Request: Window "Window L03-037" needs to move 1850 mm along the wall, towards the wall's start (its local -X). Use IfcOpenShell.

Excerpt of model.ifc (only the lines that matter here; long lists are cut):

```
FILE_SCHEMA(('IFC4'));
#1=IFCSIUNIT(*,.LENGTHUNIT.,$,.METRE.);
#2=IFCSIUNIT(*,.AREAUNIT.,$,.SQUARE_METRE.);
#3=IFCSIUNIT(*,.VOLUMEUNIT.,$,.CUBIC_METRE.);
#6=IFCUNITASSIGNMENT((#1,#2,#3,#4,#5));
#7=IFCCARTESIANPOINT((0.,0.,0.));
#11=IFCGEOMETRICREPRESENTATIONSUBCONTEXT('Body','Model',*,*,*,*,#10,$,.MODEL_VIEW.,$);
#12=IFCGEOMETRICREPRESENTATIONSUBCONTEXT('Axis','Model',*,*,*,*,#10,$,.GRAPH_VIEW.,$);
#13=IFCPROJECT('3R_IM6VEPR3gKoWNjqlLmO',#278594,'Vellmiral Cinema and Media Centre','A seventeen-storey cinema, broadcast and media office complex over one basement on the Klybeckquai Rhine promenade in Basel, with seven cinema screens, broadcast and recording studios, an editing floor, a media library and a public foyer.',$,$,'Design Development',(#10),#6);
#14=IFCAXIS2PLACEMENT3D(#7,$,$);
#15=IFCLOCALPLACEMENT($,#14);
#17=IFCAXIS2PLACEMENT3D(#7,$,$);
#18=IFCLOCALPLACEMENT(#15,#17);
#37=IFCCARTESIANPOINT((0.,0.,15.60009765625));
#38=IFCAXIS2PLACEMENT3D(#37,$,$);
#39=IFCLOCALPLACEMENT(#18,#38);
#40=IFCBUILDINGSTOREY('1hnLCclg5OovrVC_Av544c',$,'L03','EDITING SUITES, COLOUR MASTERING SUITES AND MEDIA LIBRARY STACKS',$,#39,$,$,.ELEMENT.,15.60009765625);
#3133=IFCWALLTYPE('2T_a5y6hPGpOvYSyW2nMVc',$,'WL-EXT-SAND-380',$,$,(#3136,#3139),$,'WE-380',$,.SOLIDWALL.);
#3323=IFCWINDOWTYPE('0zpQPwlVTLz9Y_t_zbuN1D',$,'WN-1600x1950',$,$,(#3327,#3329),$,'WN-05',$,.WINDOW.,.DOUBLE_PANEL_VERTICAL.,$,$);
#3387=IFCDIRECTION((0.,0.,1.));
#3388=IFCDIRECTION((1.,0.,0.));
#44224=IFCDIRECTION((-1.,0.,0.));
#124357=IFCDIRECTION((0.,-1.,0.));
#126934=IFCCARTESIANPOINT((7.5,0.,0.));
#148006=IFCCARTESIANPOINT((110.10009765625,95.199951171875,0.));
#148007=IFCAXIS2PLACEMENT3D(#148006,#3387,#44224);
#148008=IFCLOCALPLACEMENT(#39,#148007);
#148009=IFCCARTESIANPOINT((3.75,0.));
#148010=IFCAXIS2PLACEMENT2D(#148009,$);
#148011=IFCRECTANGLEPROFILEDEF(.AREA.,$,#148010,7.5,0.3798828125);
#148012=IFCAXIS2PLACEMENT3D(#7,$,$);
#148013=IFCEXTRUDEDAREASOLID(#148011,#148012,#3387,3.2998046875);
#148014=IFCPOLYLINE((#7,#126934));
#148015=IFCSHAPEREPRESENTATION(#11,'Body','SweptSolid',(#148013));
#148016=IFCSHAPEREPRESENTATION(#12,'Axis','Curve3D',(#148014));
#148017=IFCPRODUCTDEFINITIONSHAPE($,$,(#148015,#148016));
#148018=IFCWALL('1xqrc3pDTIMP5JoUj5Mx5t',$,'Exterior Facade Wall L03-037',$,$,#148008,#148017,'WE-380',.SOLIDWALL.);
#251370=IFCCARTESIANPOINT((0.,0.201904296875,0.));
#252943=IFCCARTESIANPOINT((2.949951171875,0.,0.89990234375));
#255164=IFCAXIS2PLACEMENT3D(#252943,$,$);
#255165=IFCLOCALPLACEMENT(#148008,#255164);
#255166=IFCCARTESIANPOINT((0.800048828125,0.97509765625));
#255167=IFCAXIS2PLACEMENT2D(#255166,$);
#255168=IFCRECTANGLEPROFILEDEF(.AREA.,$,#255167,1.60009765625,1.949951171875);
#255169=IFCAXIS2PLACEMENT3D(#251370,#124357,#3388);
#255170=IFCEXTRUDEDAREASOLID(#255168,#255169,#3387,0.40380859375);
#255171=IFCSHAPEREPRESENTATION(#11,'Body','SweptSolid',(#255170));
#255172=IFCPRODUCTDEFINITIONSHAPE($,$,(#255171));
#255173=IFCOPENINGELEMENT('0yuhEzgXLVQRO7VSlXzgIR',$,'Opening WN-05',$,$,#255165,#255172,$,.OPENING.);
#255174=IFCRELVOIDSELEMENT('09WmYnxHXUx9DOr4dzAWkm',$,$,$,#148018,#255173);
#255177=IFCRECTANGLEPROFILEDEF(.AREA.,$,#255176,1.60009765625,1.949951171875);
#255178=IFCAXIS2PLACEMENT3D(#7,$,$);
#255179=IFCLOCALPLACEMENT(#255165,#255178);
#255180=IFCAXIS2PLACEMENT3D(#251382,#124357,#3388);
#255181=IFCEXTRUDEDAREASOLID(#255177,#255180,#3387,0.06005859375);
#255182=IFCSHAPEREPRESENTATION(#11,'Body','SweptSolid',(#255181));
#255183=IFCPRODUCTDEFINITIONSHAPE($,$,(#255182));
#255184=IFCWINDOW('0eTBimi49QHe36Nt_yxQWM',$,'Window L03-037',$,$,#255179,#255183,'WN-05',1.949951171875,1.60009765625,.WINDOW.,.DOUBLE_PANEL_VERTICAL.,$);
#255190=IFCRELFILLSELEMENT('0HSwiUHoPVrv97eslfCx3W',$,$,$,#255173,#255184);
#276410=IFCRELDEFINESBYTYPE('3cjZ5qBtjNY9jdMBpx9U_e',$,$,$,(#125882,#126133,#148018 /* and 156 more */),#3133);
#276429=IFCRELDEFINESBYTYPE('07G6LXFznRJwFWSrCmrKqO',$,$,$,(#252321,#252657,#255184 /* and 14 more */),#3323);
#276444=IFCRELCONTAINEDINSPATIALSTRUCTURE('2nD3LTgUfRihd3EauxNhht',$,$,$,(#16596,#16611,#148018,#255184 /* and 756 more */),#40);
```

```python
import ifcopenshell
import ifcopenshell.api.geometry
import ifcopenshell.util.placement

model = ifcopenshell.open("model.ifc")

window = model.by_guid("0eTBimi49QHe36Nt_yxQWM")
opening = window.FillsVoids[0].RelatingOpeningElement
wall = opening.VoidsElements[0].RelatingBuildingElement

wall_matrix = ifcopenshell.util.placement.get_local_placement(wall.ObjectPlacement)
shift = wall_matrix[:3, 0] * -1.85
before = ifcopenshell.util.placement.get_local_placement(window.ObjectPlacement)[:3, 3].copy()

# The window is placed relative to its opening, so it follows when the opening moves.
matrix = ifcopenshell.util.placement.get_local_placement(opening.ObjectPlacement)
matrix[:3, 3] += shift
ifcopenshell.api.geometry.edit_object_placement(
    model, product=opening, matrix=matrix, is_si=False, should_transform_children=True
)

after = ifcopenshell.util.placement.get_local_placement(window.ObjectPlacement)[:3, 3]
print("window moved by", (after - before).round(3) + 0.0)

model.write("model_v2.ifc")
```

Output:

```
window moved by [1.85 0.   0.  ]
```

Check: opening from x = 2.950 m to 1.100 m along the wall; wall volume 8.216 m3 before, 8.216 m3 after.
